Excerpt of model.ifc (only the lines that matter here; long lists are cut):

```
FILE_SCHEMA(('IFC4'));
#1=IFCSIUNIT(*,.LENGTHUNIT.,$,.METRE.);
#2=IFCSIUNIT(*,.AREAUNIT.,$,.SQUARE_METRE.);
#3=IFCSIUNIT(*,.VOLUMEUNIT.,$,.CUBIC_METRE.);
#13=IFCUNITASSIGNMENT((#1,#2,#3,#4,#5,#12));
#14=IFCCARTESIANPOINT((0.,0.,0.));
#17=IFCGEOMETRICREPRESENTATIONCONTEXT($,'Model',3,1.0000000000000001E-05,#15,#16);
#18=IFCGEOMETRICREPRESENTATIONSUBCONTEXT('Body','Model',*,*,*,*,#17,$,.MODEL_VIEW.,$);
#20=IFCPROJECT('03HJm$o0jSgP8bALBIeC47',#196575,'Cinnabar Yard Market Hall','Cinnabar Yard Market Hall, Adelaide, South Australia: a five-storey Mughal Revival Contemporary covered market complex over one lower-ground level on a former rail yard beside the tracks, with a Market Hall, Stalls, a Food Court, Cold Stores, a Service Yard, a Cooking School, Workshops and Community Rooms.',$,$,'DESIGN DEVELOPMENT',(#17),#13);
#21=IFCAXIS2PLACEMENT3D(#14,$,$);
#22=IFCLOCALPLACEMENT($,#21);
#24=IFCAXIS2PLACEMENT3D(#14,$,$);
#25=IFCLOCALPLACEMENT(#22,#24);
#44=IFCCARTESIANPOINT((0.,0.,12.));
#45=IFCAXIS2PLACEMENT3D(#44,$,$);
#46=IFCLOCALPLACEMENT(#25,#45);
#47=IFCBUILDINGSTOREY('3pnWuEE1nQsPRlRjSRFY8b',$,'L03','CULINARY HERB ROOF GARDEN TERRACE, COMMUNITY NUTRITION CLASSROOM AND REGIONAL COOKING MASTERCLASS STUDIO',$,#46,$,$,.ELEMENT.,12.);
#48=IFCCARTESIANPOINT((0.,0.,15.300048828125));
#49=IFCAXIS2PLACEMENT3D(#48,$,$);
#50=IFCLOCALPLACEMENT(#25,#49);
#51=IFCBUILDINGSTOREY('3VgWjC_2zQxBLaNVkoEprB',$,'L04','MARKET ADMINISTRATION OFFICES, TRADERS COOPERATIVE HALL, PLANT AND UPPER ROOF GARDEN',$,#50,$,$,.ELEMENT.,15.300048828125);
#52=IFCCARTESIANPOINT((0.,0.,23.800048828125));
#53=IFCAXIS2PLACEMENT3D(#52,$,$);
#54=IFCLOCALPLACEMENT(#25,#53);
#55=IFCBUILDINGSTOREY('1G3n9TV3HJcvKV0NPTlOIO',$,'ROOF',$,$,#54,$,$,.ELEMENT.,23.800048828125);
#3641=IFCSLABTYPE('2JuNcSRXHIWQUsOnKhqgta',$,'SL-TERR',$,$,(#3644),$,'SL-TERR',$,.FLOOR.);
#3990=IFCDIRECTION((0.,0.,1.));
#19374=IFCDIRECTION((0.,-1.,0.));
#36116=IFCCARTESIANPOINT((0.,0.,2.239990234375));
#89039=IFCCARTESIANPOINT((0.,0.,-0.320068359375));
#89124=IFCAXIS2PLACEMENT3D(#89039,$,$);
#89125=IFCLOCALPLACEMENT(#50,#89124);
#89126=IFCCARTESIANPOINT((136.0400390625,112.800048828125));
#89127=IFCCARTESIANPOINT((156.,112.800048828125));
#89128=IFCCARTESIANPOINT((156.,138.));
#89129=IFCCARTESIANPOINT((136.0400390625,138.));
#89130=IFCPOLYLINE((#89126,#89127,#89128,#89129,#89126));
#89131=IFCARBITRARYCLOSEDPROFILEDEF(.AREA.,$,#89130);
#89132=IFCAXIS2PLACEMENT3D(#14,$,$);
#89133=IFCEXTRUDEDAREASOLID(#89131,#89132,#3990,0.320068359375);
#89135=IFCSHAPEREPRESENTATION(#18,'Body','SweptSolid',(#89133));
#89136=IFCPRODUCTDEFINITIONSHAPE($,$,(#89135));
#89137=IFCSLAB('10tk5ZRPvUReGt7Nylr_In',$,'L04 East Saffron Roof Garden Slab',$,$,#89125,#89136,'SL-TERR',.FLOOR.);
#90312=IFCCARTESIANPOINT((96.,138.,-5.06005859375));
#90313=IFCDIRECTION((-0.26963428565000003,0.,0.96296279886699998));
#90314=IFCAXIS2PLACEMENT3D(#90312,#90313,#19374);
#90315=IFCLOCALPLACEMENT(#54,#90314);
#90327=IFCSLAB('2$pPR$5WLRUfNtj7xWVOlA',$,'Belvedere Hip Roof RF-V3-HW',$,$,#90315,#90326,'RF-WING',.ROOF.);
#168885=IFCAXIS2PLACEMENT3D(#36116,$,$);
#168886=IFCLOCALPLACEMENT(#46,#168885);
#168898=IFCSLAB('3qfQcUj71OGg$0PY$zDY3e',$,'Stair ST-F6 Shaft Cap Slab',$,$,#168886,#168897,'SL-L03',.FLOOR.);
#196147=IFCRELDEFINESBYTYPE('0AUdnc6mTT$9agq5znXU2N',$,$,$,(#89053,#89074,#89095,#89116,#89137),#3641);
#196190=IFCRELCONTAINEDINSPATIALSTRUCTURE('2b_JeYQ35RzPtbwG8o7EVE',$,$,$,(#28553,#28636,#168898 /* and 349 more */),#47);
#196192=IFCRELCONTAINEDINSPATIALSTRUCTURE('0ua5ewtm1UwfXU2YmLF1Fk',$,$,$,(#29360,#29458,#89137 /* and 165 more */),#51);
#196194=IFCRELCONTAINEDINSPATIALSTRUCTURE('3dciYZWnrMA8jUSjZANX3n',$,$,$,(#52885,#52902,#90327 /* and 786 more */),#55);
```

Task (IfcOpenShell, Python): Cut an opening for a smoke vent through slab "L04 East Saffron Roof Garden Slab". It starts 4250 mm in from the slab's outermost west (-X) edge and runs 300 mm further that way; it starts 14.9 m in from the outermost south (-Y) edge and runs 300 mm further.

```python
import numpy as np
import ifcopenshell
import ifcopenshell.api.feature
import ifcopenshell.api.geometry
import ifcopenshell.api.root
import ifcopenshell.geom
import ifcopenshell.util.placement
import ifcopenshell.util.representation
import ifcopenshell.util.shape
import ifcopenshell.util.unit

model = ifcopenshell.open("model.ifc")
unit_scale = ifcopenshell.util.unit.calculate_unit_scale(model)
settings = ifcopenshell.geom.settings()


def volume(element):
    """Net volume in cubic metres, openings subtracted."""
    shape = ifcopenshell.geom.create_shape(settings, element)
    return ifcopenshell.util.shape.get_volume(shape.geometry)


slab = model.by_id(89137)
before = volume(slab)

# Extent in the slab's own axes, in metres. The edges named are its -X and -Y sides.
slab_shape = ifcopenshell.geom.create_shape(settings, slab)
vertices = ifcopenshell.util.shape.get_vertices(slab_shape.geometry)
x_min, y_min, bottom = vertices.min(axis=0)
top = vertices[:, 2].max()

opening = ifcopenshell.api.root.create_entity(model, ifc_class="IfcOpeningElement", name="Smoke vent opening", predefined_type="OPENING")
context = ifcopenshell.util.representation.get_context(model, "Model", "Body", "MODEL_VIEW")
width, depth = 0.3, 0.3
outline = [(0.0, 0.0), (width, 0.0), (width, depth), (0.0, depth), (0.0, 0.0)]
# Overshoot both faces by 50 mm so the cut is clean.
shape = ifcopenshell.api.geometry.add_slab_representation(
    model, context=context, depth=top - bottom + 0.1, polyline=outline
)
ifcopenshell.api.geometry.assign_representation(model, product=opening, representation=shape)

matrix = ifcopenshell.util.placement.get_local_placement(slab.ObjectPlacement)
matrix[:, 3] = matrix @ np.append(np.array([x_min + 4.25, y_min + 14.9, bottom - 0.05]) / unit_scale, 1.0)
ifcopenshell.api.geometry.edit_object_placement(model, product=opening, matrix=matrix, is_si=False)
ifcopenshell.api.feature.add_feature(model, feature=opening, element=slab)

after = volume(slab)

print(f"slab volume {before:.3f} -> {after:.3f} m3")

model.write("model_v2.ifc")
```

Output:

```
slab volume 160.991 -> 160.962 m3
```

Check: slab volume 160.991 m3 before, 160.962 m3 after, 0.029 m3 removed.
